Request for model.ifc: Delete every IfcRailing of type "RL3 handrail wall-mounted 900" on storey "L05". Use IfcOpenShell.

First a look at what the model holds.

```python
import ifcopenshell
import ifcopenshell.util.element

model = ifcopenshell.open("model.ifc")
print(model.schema)
storey = next(s for s in model.by_type("IfcBuildingStorey") if s.Name == "L05")
railings = [e for e in ifcopenshell.util.element.get_decomposition(storey) if e.is_a("IfcRailing")]
seen = {}
for e in railings:
    element_type = ifcopenshell.util.element.get_type(e)
    name = element_type.Name if element_type not in (None, e) else None
    seen[name] = seen.get(name, 0) + 1
for name, count in sorted(seen.items(), key=str):
    print(count, "x", name)
```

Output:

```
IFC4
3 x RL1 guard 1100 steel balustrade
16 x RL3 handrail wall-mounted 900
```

```python
import ifcopenshell
import ifcopenshell.api.root
import ifcopenshell.util.element

model = ifcopenshell.open("model.ifc")

storey = next(s for s in model.by_type("IfcBuildingStorey") if s.Name == "L05")
railings = [e for e in ifcopenshell.util.element.get_decomposition(storey) if e.is_a("IfcRailing")]
targets = [e for e in railings if (t := ifcopenshell.util.element.get_type(e)) not in (None, e) and t.Name == "RL3 handrail wall-mounted 900"]

for e in targets:
    ifcopenshell.api.root.remove_product(model, product=e)
print(len(targets), "removed")

model.write("model_rev.ifc")
```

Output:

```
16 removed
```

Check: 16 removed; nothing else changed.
